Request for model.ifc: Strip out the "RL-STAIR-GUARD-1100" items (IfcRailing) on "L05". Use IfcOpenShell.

First a look at what the model holds.

```python
import ifcopenshell
import ifcopenshell.util.element

model = ifcopenshell.open("model.ifc")
print(model.schema)
storey = next(s for s in model.by_type("IfcBuildingStorey") if s.Name == "L05")
railings = [e for e in ifcopenshell.util.element.get_decomposition(storey) if e.is_a("IfcRailing")]
seen = {}
for e in railings:
    element_type = ifcopenshell.util.element.get_type(e)
    name = element_type.Name if element_type not in (None, e) else None
    seen[name] = seen.get(name, 0) + 1
for name, count in sorted(seen.items(), key=str):
    print(count, "x", name)
```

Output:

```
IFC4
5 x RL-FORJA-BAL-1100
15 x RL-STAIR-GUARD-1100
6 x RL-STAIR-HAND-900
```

```python
import ifcopenshell
import ifcopenshell.api.root
import ifcopenshell.util.element

model = ifcopenshell.open("model.ifc")

storey = next(s for s in model.by_type("IfcBuildingStorey") if s.Name == "L05")
railings = [e for e in ifcopenshell.util.element.get_decomposition(storey) if e.is_a("IfcRailing")]
targets = [e for e in railings if (t := ifcopenshell.util.element.get_type(e)) not in (None, e) and t.Name == "RL-STAIR-GUARD-1100"]

for e in targets:
    ifcopenshell.api.root.remove_product(model, product=e)
print(len(targets), "removed")

model.write("model_edited.ifc")
```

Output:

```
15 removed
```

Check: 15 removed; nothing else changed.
